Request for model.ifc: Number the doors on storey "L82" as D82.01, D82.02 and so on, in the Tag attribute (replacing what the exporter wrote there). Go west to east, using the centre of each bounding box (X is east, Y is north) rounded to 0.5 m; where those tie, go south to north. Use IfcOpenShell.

First a look at what the model holds.

```python
import ifcopenshell
import ifcopenshell.util.element
import ifcopenshell.util.placement

model = ifcopenshell.open("model.ifc")
print(model.schema)
storey = next(s for s in model.by_type("IfcBuildingStorey") if s.Name == "L82")
doors = [e for e in ifcopenshell.util.element.get_decomposition(storey) if e.is_a("IfcDoor")]
for e in sorted(doors, key=lambda e: e.id()):
    origin = ifcopenshell.util.placement.get_local_placement(e.ObjectPlacement)[:3, 3]
    print(e.id(), e.Tag, e.Name, origin.round(2) + 0.0, sep=" | ")
```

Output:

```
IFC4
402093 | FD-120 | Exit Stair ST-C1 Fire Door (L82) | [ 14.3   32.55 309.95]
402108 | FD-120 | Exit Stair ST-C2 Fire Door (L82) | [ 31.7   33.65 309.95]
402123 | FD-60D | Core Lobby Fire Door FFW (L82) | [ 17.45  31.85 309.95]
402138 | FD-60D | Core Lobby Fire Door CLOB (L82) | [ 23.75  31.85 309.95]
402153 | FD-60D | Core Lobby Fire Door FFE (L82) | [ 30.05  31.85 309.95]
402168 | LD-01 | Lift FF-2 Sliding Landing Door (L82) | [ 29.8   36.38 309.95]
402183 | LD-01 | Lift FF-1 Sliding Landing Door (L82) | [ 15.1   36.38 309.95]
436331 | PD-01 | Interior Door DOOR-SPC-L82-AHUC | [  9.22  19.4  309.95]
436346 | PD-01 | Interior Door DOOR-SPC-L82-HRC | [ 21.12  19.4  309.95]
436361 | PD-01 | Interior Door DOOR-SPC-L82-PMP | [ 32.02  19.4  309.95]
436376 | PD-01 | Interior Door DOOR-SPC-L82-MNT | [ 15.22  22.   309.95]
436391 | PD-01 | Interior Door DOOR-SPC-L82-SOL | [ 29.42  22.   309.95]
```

```python
import ifcopenshell
import ifcopenshell.geom
import ifcopenshell.util.element
import ifcopenshell.util.shape

model = ifcopenshell.open("model.ifc")
settings = ifcopenshell.geom.settings()
settings.set("use-world-coords", True)


def centre(element):
    shape = ifcopenshell.geom.create_shape(settings, element)
    return ifcopenshell.util.shape.get_bbox_centroid(shape.geometry)


storey = next(s for s in model.by_type("IfcBuildingStorey") if s.Name == "L82")
doors = [e for e in ifcopenshell.util.element.get_decomposition(storey) if e.is_a("IfcDoor")]

# Insertion points can sit at a corner or the storey origin, so sort by the geometry (in metres).
centres = {e: centre(e) for e in doors}
doors.sort(key=lambda e: (round(centres[e][0] / 0.5), centres[e][1]))

for i, e in enumerate(doors, start=1):
    number = f"D82.{i:02d}"
    e.Tag = number
    print(e.id(), number)

model.write("model-out.ifc")
```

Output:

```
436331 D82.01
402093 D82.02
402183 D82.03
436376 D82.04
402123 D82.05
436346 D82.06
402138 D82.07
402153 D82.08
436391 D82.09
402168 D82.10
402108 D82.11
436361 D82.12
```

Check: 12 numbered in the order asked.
